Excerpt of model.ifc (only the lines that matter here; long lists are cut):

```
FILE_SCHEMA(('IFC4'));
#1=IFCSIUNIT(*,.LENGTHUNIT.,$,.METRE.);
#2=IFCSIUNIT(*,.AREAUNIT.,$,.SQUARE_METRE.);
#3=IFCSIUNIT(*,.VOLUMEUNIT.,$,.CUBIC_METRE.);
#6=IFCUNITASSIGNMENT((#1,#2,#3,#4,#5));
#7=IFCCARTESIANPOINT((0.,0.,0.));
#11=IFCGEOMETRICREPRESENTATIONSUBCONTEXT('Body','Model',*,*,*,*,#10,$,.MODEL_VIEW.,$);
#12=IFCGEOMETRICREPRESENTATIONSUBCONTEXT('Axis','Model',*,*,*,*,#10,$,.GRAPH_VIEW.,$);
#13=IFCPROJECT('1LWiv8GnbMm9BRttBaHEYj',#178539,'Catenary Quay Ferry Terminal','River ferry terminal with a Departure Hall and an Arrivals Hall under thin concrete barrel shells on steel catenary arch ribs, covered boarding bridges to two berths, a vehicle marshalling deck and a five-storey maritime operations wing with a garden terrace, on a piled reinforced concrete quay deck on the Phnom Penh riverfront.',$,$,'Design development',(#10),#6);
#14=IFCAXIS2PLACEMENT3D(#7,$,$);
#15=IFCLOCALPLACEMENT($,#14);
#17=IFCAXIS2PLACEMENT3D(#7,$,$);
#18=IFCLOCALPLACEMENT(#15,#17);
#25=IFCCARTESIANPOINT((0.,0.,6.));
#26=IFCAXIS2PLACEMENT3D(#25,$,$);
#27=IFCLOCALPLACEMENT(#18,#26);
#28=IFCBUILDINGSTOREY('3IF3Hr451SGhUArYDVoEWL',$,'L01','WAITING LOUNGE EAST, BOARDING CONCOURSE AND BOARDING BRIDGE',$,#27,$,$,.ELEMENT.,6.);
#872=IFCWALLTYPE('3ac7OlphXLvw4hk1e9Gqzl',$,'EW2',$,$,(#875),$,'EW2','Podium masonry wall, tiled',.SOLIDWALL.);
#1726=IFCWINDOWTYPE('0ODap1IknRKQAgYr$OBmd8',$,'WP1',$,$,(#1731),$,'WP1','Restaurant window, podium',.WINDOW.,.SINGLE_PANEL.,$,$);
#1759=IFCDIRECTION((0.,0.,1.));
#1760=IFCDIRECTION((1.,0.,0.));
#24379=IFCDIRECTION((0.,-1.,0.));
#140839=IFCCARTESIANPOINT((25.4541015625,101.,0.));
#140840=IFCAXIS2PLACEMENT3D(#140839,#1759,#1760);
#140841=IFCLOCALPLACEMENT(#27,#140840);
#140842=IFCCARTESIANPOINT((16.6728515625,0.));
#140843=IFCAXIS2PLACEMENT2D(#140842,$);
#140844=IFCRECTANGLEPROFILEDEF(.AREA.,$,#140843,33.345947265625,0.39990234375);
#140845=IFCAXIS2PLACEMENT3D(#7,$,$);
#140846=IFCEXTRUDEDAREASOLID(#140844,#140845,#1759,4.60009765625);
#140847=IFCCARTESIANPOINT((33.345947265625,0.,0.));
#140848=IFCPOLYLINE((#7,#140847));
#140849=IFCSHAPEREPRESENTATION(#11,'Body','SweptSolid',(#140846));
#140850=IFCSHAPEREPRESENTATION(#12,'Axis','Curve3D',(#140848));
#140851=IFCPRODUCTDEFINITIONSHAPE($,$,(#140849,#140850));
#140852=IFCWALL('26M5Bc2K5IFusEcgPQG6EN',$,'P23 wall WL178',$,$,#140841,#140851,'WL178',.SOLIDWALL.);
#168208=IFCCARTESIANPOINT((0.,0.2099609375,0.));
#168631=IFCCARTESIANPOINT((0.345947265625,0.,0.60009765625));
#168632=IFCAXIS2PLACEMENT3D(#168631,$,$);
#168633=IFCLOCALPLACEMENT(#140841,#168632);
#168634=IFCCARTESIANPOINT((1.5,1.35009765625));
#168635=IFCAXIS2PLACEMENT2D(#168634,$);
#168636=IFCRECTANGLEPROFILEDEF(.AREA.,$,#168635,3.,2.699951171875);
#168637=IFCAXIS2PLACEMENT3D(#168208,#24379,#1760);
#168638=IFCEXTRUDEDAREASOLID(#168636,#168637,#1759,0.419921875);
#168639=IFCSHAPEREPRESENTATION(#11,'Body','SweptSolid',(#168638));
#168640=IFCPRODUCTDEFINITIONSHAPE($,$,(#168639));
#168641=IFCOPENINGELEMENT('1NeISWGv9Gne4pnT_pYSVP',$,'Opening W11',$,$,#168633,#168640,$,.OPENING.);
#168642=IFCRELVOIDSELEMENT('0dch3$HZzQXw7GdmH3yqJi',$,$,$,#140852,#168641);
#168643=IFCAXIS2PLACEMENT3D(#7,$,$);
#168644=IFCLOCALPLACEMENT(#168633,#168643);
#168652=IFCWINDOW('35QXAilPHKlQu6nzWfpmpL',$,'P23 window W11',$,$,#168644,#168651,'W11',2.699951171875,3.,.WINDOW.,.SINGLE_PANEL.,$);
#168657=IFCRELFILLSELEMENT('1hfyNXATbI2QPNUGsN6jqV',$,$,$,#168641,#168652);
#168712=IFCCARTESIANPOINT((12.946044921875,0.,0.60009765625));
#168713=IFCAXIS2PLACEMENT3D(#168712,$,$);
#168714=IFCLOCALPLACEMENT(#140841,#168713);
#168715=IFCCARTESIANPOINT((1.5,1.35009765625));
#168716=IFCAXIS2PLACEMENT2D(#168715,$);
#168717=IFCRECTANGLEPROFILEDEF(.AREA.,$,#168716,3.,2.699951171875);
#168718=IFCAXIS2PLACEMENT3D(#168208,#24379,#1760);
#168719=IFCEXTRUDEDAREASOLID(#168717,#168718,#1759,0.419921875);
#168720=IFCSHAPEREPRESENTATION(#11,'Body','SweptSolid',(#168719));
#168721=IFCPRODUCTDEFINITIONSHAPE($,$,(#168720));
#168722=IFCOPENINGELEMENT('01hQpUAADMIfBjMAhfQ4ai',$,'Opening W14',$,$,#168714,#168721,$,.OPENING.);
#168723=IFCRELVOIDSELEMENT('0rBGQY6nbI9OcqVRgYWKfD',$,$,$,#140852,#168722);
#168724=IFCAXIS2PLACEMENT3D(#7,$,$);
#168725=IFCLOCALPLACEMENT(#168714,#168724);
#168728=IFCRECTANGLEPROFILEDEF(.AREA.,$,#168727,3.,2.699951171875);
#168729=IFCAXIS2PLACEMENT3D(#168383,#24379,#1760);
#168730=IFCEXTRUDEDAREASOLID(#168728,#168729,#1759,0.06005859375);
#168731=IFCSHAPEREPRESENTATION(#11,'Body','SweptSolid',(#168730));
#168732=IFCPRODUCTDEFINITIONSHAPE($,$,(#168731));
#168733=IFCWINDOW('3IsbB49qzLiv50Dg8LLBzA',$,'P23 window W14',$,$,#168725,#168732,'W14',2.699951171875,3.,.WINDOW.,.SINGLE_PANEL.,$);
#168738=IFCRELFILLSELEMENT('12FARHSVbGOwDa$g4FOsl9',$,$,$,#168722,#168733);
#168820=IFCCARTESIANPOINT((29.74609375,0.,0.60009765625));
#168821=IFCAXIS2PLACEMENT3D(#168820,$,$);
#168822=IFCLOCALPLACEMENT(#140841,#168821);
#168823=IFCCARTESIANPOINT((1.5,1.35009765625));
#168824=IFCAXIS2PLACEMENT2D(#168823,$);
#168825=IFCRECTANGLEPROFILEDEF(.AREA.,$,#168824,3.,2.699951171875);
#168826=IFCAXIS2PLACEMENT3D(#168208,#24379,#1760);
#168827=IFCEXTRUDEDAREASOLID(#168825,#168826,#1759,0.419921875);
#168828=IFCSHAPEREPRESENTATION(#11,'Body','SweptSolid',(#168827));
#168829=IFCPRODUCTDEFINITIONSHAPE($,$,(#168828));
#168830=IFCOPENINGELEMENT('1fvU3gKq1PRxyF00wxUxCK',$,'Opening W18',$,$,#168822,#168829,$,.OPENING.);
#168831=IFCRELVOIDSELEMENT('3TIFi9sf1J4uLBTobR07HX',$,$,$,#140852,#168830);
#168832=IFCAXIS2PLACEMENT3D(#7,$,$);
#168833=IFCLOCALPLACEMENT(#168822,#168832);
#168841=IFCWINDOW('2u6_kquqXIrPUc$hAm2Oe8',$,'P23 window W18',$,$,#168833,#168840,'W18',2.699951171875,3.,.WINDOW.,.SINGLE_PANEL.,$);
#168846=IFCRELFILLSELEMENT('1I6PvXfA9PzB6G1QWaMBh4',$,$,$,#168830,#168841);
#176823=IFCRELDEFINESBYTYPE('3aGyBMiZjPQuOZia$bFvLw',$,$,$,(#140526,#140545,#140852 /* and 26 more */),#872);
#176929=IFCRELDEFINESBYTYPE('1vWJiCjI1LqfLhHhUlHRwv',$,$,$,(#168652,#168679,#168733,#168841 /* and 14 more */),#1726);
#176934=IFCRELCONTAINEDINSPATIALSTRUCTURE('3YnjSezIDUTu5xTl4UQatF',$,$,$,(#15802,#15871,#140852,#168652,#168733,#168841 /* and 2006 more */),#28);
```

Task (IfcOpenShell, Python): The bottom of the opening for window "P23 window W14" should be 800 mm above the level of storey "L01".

```python
import numpy as np
import ifcopenshell
import ifcopenshell.api.geometry
import ifcopenshell.geom
import ifcopenshell.util.element
import ifcopenshell.util.placement
import ifcopenshell.util.shape
import ifcopenshell.util.unit

model = ifcopenshell.open("model.ifc")
unit_scale = ifcopenshell.util.unit.calculate_unit_scale(model)

window = model.by_guid("3IsbB49qzLiv50Dg8LLBzA")
opening = window.FillsVoids[0].RelatingOpeningElement
storey = ifcopenshell.util.element.get_container(window, ifc_class="IfcBuildingStorey")
level = ifcopenshell.util.placement.get_local_placement(storey.ObjectPlacement)[2, 3]

# The opening's origin need not be at the sill, so measure its lowest point.
shape = ifcopenshell.geom.create_shape(ifcopenshell.geom.settings(), opening)
bottom = ifcopenshell.util.shape.get_shape_bottom_elevation(shape, shape.geometry) / unit_scale
dz = level + 0.8 / unit_scale - bottom

shift = np.array([0.0, 0.0, dz])
# The window is placed relative to its opening, so it follows when the opening moves.
matrix = ifcopenshell.util.placement.get_local_placement(opening.ObjectPlacement)
matrix[:3, 3] += shift
ifcopenshell.api.geometry.edit_object_placement(
    model, product=opening, matrix=matrix, is_si=False, should_transform_children=True
)

print(f"moved by {dz * unit_scale:+.3f} m")

model.write("model-out.ifc")
```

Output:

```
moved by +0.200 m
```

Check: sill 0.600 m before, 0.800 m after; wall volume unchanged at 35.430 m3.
